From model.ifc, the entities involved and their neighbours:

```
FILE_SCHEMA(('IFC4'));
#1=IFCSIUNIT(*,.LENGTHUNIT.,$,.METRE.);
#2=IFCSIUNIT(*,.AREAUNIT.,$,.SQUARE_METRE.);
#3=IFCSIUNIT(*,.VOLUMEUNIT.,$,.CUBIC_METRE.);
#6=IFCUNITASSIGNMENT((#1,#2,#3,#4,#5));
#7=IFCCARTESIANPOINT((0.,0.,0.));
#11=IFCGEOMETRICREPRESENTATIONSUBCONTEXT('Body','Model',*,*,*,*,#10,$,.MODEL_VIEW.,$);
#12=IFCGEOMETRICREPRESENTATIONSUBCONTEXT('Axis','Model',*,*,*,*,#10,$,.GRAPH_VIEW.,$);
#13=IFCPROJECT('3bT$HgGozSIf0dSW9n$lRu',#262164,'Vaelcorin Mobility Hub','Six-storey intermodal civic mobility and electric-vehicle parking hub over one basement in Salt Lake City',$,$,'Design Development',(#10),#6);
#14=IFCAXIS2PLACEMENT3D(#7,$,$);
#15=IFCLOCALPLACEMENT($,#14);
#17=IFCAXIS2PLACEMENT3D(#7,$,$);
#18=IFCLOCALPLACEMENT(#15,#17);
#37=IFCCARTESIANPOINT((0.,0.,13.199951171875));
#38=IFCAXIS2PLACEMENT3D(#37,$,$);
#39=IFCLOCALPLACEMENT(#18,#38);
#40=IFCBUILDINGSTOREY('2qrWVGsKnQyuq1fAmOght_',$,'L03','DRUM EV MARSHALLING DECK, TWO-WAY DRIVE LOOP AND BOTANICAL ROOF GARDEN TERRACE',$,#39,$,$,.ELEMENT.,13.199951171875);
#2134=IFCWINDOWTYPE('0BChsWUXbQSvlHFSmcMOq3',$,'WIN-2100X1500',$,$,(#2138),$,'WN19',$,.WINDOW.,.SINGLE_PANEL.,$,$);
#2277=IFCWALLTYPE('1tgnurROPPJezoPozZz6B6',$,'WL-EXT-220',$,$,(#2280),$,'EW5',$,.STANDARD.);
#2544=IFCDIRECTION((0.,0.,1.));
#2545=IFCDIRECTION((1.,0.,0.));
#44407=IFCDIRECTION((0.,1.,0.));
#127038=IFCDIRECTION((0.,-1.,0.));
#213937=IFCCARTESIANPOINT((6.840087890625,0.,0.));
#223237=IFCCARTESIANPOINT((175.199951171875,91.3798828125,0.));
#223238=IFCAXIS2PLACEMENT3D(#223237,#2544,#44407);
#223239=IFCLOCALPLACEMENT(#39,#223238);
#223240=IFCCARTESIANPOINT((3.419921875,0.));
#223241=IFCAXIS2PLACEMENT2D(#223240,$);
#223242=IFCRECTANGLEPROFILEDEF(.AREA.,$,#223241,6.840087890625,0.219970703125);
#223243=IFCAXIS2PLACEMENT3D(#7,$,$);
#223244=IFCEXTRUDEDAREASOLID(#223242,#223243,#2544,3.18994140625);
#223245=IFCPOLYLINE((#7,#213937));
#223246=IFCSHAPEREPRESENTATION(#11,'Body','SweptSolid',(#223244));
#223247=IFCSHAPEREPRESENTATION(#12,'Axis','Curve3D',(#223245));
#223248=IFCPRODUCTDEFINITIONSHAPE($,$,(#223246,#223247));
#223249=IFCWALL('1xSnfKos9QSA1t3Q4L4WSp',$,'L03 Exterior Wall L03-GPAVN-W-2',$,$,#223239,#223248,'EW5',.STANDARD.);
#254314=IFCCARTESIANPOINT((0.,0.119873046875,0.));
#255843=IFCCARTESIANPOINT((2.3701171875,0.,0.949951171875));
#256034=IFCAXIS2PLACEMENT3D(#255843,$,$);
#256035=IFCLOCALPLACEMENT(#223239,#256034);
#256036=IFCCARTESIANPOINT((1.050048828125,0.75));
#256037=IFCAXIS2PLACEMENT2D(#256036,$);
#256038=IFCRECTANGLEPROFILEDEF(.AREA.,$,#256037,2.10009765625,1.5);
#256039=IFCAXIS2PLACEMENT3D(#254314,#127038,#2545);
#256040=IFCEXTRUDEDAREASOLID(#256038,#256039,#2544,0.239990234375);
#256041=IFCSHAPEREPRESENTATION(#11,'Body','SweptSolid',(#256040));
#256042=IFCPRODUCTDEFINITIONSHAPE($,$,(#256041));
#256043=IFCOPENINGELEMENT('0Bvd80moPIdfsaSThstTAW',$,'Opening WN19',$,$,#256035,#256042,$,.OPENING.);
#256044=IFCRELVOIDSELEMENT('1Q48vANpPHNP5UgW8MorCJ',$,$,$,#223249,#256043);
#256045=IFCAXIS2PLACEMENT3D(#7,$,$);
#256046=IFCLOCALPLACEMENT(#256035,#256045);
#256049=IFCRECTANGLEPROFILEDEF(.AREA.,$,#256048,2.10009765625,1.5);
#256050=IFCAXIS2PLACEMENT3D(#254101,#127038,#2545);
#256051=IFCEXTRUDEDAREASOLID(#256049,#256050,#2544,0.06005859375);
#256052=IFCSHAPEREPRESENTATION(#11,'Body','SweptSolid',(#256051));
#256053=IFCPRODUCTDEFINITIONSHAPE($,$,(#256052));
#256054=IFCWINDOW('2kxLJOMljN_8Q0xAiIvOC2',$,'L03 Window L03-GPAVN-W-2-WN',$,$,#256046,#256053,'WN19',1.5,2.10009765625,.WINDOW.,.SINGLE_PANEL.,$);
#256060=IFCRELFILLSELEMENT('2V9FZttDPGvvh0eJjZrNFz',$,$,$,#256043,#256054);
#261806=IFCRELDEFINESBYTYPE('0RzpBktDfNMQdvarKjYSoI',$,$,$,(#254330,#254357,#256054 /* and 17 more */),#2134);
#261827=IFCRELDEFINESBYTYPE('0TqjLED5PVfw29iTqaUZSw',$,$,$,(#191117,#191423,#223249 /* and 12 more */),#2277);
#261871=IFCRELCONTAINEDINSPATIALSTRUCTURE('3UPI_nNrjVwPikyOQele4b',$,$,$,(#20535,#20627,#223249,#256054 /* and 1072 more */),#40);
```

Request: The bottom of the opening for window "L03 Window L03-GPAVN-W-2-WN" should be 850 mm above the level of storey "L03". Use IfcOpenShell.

```python
import numpy as np
import ifcopenshell
import ifcopenshell.api.geometry
import ifcopenshell.geom
import ifcopenshell.util.element
import ifcopenshell.util.placement
import ifcopenshell.util.shape
import ifcopenshell.util.unit

model = ifcopenshell.open("model.ifc")
unit_scale = ifcopenshell.util.unit.calculate_unit_scale(model)

window = model.by_id(256054)
opening = window.FillsVoids[0].RelatingOpeningElement
storey = ifcopenshell.util.element.get_container(window, ifc_class="IfcBuildingStorey")
level = ifcopenshell.util.placement.get_local_placement(storey.ObjectPlacement)[2, 3]

# The opening's origin need not be at the sill, so measure its lowest point.
shape = ifcopenshell.geom.create_shape(ifcopenshell.geom.settings(), opening)
bottom = ifcopenshell.util.shape.get_shape_bottom_elevation(shape, shape.geometry) / unit_scale
dz = level + 0.85 - bottom

shift = np.array([0.0, 0.0, dz])
# The window is placed relative to its opening, so it follows when the opening moves.
matrix = ifcopenshell.util.placement.get_local_placement(opening.ObjectPlacement)
matrix[:3, 3] += shift
ifcopenshell.api.geometry.edit_object_placement(
    model, product=opening, matrix=matrix, is_si=False, should_transform_children=True
)

print(f"moved by {dz * unit_scale:+.3f} m")

model.write("model_edited.ifc")
```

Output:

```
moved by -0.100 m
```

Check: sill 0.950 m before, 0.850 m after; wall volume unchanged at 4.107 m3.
